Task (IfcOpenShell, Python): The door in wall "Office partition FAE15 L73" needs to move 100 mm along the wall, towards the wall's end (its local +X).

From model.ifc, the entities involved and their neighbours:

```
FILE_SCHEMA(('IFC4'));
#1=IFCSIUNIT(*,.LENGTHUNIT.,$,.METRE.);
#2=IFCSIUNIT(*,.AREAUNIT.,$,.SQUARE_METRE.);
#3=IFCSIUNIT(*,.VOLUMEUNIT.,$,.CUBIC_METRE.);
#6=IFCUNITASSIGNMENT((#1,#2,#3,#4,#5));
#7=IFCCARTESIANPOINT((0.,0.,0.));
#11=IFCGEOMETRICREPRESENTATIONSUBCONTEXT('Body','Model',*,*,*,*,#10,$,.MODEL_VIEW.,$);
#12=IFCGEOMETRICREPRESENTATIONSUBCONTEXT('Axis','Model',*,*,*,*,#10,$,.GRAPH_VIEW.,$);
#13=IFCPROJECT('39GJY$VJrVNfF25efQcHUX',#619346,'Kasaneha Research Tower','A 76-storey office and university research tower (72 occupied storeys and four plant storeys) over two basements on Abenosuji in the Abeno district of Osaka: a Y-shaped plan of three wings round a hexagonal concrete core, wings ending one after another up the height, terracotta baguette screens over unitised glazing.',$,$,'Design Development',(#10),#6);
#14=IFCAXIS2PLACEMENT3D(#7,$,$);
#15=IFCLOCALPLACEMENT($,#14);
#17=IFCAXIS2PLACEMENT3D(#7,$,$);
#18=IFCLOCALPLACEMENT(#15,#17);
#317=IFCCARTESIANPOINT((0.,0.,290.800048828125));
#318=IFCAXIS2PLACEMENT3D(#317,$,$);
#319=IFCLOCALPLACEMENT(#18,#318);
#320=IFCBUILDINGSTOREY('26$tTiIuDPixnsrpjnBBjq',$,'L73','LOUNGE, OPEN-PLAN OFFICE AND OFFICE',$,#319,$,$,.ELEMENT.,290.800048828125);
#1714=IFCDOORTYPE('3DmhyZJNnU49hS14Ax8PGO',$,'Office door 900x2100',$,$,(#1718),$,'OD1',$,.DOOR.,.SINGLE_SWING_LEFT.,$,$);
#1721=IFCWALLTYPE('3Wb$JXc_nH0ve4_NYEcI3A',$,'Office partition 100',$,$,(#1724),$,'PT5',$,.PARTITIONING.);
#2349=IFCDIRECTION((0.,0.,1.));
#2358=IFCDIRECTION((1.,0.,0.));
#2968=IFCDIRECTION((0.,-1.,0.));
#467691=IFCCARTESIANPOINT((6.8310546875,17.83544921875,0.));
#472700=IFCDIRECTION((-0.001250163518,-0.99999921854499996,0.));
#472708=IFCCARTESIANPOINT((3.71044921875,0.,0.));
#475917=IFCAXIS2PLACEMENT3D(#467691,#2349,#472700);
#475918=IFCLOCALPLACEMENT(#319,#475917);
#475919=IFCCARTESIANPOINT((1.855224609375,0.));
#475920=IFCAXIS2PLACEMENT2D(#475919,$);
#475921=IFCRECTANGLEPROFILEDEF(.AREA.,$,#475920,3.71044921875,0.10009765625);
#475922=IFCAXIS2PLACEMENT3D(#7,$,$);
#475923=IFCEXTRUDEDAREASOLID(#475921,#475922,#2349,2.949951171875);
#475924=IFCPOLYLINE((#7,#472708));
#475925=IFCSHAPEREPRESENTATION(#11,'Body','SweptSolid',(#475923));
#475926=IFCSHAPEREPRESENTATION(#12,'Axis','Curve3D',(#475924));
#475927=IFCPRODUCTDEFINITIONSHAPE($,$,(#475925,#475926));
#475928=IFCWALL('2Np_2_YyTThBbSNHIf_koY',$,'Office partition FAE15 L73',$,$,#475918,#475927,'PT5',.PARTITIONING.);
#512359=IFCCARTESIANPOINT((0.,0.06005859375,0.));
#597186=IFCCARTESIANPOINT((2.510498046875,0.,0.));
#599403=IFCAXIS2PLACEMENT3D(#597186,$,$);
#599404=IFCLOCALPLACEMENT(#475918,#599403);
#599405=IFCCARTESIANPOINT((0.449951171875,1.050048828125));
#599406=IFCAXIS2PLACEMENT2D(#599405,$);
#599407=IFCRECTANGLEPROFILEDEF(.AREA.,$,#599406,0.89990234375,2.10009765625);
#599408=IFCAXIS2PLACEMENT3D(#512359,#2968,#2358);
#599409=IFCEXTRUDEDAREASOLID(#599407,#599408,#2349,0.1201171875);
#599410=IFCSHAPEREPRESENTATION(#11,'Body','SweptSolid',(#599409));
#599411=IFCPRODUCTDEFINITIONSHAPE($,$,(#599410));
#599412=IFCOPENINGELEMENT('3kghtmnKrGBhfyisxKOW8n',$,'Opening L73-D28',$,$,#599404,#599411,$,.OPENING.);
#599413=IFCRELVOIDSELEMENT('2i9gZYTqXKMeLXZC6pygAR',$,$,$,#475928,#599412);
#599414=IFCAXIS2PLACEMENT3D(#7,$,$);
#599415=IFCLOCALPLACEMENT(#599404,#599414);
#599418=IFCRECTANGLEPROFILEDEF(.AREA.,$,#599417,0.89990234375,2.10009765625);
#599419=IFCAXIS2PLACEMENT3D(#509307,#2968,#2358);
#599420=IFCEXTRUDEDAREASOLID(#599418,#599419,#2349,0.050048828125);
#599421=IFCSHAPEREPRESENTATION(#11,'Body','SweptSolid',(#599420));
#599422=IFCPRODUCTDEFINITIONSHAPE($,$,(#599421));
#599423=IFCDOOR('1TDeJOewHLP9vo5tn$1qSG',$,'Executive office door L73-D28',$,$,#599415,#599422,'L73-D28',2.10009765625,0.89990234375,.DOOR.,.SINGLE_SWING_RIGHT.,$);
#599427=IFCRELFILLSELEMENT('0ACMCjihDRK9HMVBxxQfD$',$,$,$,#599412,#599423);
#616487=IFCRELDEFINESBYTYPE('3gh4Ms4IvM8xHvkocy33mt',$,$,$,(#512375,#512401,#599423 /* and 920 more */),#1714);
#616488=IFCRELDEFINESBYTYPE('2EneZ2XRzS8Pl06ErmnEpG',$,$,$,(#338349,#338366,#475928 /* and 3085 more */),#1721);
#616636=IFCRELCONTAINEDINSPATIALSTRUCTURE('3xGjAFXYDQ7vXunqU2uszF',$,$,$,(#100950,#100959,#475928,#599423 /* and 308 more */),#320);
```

```python
import ifcopenshell
import ifcopenshell.api.geometry
import ifcopenshell.util.placement

model = ifcopenshell.open("model.ifc")

door = model.by_id(599423)
opening = door.FillsVoids[0].RelatingOpeningElement
wall = opening.VoidsElements[0].RelatingBuildingElement

wall_matrix = ifcopenshell.util.placement.get_local_placement(wall.ObjectPlacement)
shift = wall_matrix[:3, 0] * 0.1
before = ifcopenshell.util.placement.get_local_placement(door.ObjectPlacement)[:3, 3].copy()

# The door is placed relative to its opening, so it follows when the opening moves.
matrix = ifcopenshell.util.placement.get_local_placement(opening.ObjectPlacement)
matrix[:3, 3] += shift
ifcopenshell.api.geometry.edit_object_placement(
    model, product=opening, matrix=matrix, is_si=False, should_transform_children=True
)

after = ifcopenshell.util.placement.get_local_placement(door.ObjectPlacement)[:3, 3]
print("door moved by", (after - before).round(3) + 0.0)

model.write("model_updated.ifc")
```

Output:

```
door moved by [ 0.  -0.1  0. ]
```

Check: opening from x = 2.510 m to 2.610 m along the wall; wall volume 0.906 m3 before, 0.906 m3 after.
